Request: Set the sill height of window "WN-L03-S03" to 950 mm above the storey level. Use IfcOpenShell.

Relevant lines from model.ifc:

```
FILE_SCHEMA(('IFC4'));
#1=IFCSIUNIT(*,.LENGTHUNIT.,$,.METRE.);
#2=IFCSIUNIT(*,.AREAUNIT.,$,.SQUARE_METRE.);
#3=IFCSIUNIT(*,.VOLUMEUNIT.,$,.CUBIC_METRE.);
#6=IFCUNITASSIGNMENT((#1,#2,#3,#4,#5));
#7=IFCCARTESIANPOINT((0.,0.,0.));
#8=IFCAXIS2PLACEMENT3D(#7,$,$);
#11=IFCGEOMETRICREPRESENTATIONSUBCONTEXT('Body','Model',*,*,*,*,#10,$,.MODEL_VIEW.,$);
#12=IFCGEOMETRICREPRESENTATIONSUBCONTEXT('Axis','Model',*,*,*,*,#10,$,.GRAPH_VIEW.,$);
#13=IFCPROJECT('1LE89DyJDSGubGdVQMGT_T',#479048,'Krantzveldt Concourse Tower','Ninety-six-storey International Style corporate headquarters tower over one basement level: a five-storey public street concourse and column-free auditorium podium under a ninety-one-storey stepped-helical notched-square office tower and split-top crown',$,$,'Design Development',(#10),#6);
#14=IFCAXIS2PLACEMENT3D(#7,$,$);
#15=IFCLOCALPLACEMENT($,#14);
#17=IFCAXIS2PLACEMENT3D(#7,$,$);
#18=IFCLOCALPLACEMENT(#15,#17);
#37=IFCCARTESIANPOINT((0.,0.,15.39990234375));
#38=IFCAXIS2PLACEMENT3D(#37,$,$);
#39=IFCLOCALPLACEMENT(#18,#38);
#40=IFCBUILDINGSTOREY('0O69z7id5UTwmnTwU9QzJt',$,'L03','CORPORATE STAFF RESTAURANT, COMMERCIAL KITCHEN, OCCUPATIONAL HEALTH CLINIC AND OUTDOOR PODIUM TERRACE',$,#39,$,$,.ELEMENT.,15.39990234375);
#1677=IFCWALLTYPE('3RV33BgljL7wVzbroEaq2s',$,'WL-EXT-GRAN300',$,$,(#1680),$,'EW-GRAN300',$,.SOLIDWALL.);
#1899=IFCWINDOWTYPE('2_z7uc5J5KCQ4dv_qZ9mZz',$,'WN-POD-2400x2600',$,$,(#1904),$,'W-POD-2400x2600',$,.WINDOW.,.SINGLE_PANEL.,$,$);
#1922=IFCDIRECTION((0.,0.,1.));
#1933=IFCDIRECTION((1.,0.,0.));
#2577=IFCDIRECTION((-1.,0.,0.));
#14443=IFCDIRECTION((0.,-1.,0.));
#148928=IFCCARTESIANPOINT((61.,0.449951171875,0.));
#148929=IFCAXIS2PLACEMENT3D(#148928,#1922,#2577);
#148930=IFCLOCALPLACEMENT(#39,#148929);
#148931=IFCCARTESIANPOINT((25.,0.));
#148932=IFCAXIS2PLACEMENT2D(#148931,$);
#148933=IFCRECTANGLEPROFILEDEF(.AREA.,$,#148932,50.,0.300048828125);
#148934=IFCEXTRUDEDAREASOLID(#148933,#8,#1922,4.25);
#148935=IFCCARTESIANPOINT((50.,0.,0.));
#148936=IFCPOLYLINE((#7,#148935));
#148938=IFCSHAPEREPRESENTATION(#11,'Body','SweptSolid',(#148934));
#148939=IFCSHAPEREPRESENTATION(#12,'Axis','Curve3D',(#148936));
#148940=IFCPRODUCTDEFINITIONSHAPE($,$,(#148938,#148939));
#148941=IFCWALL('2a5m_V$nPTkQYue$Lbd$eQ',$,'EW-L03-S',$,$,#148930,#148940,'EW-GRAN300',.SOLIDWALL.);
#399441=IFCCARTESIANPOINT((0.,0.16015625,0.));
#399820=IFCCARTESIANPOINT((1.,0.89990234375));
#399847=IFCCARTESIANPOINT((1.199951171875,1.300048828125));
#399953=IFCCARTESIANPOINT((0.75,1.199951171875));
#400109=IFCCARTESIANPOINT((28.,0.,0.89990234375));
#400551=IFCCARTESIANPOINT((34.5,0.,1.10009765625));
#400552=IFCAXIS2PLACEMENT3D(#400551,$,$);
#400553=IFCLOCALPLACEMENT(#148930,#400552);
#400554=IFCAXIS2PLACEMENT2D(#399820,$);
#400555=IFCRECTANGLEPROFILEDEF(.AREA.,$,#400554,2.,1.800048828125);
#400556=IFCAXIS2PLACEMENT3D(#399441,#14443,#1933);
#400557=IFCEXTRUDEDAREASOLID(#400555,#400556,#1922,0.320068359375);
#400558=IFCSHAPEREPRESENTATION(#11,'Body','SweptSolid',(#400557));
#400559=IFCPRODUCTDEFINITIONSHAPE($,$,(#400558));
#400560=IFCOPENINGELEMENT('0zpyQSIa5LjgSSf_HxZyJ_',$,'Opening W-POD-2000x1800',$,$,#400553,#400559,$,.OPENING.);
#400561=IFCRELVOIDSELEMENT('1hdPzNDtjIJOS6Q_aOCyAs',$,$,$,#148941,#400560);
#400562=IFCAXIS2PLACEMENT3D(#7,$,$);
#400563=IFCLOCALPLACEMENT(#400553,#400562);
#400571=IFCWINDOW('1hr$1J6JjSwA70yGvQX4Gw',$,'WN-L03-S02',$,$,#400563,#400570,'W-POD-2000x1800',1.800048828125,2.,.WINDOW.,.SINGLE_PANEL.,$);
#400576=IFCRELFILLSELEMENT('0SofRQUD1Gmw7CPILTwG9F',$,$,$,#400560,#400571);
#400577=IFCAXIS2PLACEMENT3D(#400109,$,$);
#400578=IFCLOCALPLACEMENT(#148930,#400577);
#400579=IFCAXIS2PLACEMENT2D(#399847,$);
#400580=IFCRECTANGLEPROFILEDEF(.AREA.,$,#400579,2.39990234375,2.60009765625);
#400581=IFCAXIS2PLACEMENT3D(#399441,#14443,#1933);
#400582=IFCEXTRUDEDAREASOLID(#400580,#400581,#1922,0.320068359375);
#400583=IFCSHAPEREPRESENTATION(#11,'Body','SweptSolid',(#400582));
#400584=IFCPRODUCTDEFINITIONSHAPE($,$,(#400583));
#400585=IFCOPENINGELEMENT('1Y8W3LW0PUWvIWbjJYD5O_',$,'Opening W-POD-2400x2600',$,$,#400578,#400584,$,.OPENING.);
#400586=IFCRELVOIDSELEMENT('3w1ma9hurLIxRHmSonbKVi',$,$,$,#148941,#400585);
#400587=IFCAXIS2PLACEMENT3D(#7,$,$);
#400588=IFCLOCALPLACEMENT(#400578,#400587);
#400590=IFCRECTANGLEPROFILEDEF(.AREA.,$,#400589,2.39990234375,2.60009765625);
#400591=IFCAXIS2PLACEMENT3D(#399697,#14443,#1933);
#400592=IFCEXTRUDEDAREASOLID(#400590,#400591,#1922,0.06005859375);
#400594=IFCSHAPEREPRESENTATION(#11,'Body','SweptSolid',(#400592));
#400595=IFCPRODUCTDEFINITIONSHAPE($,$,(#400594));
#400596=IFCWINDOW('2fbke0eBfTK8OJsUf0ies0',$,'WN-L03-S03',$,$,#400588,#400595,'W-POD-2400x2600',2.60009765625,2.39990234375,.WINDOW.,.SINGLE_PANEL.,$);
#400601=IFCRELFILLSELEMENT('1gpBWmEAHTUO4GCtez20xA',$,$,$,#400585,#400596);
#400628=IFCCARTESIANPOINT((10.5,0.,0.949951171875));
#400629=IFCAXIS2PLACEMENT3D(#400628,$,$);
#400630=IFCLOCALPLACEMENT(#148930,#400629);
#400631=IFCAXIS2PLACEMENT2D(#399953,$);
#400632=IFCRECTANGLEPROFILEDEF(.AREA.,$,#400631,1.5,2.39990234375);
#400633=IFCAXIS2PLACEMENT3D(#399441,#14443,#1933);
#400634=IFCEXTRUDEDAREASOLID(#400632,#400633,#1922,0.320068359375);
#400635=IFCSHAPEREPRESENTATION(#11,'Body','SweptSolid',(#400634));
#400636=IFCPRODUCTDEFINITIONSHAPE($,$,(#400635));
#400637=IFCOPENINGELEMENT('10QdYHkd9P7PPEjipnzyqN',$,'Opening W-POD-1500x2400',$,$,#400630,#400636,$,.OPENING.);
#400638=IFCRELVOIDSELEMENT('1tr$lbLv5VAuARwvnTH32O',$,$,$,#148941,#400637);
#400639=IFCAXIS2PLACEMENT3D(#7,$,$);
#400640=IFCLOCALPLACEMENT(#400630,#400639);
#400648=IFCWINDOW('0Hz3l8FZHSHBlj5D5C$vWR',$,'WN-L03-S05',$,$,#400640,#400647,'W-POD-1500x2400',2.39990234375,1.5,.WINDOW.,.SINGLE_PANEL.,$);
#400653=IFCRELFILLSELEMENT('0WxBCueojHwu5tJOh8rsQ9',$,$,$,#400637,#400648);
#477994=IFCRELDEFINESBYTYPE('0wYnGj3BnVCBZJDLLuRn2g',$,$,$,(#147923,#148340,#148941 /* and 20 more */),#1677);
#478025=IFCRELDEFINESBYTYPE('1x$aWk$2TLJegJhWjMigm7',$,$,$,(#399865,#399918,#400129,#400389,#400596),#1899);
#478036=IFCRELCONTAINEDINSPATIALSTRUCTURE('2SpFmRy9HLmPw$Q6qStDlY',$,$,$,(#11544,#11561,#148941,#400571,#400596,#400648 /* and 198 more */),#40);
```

```python
import numpy as np
import ifcopenshell
import ifcopenshell.api.geometry
import ifcopenshell.geom
import ifcopenshell.util.element
import ifcopenshell.util.placement
import ifcopenshell.util.shape
import ifcopenshell.util.unit

model = ifcopenshell.open("model.ifc")
unit_scale = ifcopenshell.util.unit.calculate_unit_scale(model)

window = model.by_guid("2fbke0eBfTK8OJsUf0ies0")
opening = window.FillsVoids[0].RelatingOpeningElement
storey = ifcopenshell.util.element.get_container(window, ifc_class="IfcBuildingStorey")
level = ifcopenshell.util.placement.get_local_placement(storey.ObjectPlacement)[2, 3]

# The opening's origin need not be at the sill, so measure its lowest point.
shape = ifcopenshell.geom.create_shape(ifcopenshell.geom.settings(), opening)
bottom = ifcopenshell.util.shape.get_shape_bottom_elevation(shape, shape.geometry) / unit_scale
dz = level + 0.95 / unit_scale - bottom

shift = np.array([0.0, 0.0, dz])
# The window is placed relative to its opening, so it follows when the opening moves.
matrix = ifcopenshell.util.placement.get_local_placement(opening.ObjectPlacement)
matrix[:3, 3] += shift
ifcopenshell.api.geometry.edit_object_placement(
    model, product=opening, matrix=matrix, is_si=False, should_transform_children=True
)

print(f"moved by {dz * unit_scale:+.3f} m")

model.write("model_rev.ifc")
```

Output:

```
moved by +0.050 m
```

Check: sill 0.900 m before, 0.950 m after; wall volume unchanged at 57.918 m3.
